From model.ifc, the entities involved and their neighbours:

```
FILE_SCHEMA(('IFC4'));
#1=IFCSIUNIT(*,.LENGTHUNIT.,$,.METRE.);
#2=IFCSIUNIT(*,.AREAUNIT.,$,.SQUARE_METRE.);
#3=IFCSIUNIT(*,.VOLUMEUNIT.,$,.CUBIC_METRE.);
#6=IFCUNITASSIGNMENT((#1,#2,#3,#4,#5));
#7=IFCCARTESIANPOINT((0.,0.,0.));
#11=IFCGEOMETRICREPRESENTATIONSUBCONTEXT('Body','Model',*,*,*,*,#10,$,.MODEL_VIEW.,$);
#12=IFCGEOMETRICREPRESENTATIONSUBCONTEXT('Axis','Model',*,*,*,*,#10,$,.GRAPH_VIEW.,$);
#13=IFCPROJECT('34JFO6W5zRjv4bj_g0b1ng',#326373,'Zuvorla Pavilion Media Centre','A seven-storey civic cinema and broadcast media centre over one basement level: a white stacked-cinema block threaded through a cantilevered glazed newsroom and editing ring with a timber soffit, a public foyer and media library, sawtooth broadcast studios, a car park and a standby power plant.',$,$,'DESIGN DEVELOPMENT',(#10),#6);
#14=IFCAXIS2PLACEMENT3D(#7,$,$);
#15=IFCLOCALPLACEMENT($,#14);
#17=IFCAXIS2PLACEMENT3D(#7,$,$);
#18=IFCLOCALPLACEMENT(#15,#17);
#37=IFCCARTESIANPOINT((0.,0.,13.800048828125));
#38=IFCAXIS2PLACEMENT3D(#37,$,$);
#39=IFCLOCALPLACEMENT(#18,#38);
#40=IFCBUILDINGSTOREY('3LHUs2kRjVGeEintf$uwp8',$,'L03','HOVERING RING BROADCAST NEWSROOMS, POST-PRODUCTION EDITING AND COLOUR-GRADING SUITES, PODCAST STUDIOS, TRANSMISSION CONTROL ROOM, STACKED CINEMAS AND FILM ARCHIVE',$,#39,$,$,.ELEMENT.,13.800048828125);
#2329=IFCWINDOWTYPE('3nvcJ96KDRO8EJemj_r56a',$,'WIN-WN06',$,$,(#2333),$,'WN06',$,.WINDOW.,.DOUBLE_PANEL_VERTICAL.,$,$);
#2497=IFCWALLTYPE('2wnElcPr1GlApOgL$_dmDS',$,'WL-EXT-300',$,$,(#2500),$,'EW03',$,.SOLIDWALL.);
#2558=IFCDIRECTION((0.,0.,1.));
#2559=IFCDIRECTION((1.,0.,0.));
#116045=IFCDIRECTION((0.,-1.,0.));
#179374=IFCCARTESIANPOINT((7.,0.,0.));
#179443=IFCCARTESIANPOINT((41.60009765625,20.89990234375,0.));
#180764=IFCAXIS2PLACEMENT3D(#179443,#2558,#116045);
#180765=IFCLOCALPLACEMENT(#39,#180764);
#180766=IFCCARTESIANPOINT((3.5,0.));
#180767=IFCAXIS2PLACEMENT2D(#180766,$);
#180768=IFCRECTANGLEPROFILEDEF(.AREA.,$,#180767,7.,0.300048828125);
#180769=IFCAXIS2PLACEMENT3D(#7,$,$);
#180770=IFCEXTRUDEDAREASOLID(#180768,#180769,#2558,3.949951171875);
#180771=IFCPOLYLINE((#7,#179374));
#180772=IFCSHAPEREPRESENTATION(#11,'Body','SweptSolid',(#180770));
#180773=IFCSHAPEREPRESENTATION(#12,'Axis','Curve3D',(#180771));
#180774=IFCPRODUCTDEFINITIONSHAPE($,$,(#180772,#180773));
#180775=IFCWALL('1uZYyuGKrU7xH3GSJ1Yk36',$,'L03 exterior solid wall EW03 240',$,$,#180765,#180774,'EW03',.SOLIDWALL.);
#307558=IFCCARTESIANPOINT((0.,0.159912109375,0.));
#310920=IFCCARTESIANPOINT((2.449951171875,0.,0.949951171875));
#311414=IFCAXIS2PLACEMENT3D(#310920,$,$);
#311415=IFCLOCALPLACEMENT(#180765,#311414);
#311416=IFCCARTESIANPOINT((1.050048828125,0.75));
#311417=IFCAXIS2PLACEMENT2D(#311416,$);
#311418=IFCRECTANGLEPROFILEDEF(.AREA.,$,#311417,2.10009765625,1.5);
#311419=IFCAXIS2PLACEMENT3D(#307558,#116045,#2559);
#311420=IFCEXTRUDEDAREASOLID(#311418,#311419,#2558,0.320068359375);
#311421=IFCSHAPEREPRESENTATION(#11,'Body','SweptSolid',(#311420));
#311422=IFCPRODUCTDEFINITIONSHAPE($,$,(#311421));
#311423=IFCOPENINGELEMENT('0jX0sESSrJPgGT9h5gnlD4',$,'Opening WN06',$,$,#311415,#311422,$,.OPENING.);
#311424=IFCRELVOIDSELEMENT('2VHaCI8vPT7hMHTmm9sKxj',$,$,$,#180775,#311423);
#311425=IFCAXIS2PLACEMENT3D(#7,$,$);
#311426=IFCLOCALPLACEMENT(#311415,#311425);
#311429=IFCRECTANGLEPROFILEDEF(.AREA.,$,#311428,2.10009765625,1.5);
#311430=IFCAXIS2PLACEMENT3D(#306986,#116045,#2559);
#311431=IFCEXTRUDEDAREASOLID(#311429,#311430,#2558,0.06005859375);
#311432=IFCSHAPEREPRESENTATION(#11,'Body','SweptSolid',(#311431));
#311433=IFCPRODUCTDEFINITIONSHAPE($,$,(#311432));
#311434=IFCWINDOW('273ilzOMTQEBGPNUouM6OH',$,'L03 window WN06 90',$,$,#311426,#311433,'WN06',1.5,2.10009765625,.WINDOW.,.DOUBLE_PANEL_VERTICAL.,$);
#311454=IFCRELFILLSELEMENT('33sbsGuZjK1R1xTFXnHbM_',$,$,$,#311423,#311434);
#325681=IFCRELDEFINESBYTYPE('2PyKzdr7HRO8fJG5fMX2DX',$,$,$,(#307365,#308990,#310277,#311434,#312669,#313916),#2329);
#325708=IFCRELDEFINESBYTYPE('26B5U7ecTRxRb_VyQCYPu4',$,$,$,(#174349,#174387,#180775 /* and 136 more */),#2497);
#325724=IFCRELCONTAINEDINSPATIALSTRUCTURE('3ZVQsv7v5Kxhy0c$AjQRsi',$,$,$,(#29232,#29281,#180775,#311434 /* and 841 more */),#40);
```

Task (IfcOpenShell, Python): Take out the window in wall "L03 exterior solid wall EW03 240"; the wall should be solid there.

```python
import ifcopenshell
import ifcopenshell.api.feature
import ifcopenshell.api.root
import ifcopenshell.geom
import ifcopenshell.util.shape

model = ifcopenshell.open("model.ifc")
settings = ifcopenshell.geom.settings()


def volume(element):
    """Net volume in cubic metres, openings subtracted."""
    shape = ifcopenshell.geom.create_shape(settings, element)
    return ifcopenshell.util.shape.get_volume(shape.geometry)


window = model.by_id(311434)
opening = window.FillsVoids[0].RelatingOpeningElement
wall = opening.VoidsElements[0].RelatingBuildingElement
before = volume(wall)

ifcopenshell.api.root.remove_product(model, product=window)
ifcopenshell.api.feature.remove_feature(model, feature=opening)

after = volume(wall)

print(f"wall volume {before:.3f} -> {after:.3f} m3")

model.write("model_edited.ifc")
```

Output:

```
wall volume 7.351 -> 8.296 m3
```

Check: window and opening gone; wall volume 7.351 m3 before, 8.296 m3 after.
